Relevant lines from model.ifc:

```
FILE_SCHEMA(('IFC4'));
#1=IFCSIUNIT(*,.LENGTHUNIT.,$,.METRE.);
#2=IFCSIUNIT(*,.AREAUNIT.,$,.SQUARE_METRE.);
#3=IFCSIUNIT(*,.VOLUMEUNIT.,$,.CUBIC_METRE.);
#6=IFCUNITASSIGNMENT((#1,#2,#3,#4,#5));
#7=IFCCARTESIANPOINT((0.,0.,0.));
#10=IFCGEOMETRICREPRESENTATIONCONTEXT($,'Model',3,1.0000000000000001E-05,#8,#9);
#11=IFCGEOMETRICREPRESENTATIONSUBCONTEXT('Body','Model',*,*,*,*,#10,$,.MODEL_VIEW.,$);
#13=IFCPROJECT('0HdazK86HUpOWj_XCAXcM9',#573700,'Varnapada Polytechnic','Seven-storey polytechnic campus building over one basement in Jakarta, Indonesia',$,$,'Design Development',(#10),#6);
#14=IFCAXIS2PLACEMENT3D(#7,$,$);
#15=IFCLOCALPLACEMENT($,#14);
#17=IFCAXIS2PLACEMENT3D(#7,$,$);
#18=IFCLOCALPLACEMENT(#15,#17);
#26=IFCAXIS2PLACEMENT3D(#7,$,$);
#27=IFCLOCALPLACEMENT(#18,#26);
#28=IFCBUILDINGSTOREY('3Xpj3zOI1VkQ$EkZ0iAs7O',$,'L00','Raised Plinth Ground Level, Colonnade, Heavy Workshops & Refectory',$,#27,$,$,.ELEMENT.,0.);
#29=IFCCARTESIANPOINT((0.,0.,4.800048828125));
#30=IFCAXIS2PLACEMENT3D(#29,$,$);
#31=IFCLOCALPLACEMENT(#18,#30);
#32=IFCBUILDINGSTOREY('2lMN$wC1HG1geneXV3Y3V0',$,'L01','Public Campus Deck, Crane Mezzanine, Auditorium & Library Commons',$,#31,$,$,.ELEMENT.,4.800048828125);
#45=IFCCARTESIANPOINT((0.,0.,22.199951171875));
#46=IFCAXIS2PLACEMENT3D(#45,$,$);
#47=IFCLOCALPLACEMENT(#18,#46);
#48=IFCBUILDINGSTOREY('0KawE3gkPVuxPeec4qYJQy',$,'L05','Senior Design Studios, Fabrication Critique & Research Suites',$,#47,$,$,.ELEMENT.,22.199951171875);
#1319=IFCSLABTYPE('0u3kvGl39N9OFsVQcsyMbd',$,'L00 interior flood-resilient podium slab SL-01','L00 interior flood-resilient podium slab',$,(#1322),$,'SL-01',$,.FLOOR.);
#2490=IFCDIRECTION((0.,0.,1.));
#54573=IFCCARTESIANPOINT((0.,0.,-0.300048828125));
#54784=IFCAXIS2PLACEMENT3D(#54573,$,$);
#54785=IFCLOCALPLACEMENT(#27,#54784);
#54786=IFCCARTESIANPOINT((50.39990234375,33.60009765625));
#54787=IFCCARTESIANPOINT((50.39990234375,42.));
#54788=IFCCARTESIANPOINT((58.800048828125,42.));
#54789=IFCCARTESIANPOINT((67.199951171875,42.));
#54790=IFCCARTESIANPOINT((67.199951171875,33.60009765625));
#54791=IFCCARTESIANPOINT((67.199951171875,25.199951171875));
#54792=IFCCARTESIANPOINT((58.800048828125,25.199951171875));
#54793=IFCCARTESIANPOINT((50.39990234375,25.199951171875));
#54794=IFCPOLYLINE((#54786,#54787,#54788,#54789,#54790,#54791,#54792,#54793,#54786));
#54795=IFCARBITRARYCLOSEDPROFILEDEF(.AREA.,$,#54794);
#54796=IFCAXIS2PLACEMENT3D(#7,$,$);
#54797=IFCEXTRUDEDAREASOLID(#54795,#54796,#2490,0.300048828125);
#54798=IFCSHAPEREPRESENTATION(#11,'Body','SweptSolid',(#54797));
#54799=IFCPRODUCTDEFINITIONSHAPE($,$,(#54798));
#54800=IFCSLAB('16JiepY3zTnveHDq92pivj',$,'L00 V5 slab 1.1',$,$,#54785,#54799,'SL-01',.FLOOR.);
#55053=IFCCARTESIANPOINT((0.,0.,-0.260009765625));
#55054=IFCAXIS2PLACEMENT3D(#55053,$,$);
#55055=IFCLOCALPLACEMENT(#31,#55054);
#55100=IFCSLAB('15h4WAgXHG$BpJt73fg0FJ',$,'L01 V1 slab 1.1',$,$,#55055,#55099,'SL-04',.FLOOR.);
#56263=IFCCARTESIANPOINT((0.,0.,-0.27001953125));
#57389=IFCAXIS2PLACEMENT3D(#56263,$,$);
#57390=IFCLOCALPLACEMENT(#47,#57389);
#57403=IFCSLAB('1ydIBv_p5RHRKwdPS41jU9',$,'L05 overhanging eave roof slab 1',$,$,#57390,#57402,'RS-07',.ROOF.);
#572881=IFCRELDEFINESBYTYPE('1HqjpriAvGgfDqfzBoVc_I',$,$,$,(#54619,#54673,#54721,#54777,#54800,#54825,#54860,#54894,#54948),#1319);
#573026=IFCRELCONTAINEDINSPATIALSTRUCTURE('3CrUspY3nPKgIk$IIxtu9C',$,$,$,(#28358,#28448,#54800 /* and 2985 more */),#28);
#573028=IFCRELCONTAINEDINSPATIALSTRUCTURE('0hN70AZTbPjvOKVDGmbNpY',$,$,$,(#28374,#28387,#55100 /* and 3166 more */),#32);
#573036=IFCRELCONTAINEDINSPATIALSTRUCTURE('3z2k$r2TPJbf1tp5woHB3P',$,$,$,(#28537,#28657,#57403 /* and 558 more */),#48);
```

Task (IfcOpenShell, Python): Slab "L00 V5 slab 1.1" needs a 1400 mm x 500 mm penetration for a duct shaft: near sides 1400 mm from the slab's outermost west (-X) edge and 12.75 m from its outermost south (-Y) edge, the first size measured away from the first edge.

```python
import numpy as np
import ifcopenshell
import ifcopenshell.api.feature
import ifcopenshell.api.geometry
import ifcopenshell.api.root
import ifcopenshell.geom
import ifcopenshell.util.placement
import ifcopenshell.util.representation
import ifcopenshell.util.shape
import ifcopenshell.util.unit

model = ifcopenshell.open("model.ifc")
unit_scale = ifcopenshell.util.unit.calculate_unit_scale(model)
settings = ifcopenshell.geom.settings()


def volume(element):
    """Net volume in cubic metres, openings subtracted."""
    shape = ifcopenshell.geom.create_shape(settings, element)
    return ifcopenshell.util.shape.get_volume(shape.geometry)


slab = model.by_guid("16JiepY3zTnveHDq92pivj")
before = volume(slab)

# Extent in the slab's own axes, in metres. The edges named are its -X and -Y sides.
slab_shape = ifcopenshell.geom.create_shape(settings, slab)
vertices = ifcopenshell.util.shape.get_vertices(slab_shape.geometry)
x_min, y_min, bottom = vertices.min(axis=0)
top = vertices[:, 2].max()

opening = ifcopenshell.api.root.create_entity(model, ifc_class="IfcOpeningElement", name="Duct shaft opening", predefined_type="OPENING")
context = ifcopenshell.util.representation.get_context(model, "Model", "Body", "MODEL_VIEW")
width, depth = 1.4, 0.5
outline = [(0.0, 0.0), (width, 0.0), (width, depth), (0.0, depth), (0.0, 0.0)]
# Overshoot both faces by 50 mm so the cut is clean.
shape = ifcopenshell.api.geometry.add_slab_representation(
    model, context=context, depth=top - bottom + 0.1, polyline=outline
)
ifcopenshell.api.geometry.assign_representation(model, product=opening, representation=shape)

matrix = ifcopenshell.util.placement.get_local_placement(slab.ObjectPlacement)
matrix[:, 3] = matrix @ np.append(np.array([x_min + 1.4, y_min + 12.75, bottom - 0.05]) / unit_scale, 1.0)
ifcopenshell.api.geometry.edit_object_placement(model, product=opening, matrix=matrix, is_si=False)
ifcopenshell.api.feature.add_feature(model, feature=opening, element=slab)

after = volume(slab)

print(f"slab volume {before:.3f} -> {after:.3f} m3")

model.write("model_rev.ifc")
```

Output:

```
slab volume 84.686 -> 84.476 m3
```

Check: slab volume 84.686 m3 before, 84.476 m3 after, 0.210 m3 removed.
